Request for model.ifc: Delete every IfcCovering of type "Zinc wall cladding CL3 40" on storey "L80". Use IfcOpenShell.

First a look at what the model holds.

```python
import ifcopenshell
import ifcopenshell.util.element

model = ifcopenshell.open("model.ifc")
print(model.schema)
storey = next(s for s in model.by_type("IfcBuildingStorey") if s.Name == "L80")
coverings = [e for e in ifcopenshell.util.element.get_decomposition(storey) if e.is_a("IfcCovering")]
seen = {}
for e in coverings:
    element_type = ifcopenshell.util.element.get_type(e)
    name = element_type.Name if element_type not in (None, e) else None
    seen[name] = seen.get(name, 0) + 1
for name, count in sorted(seen.items(), key=str):
    print(count, "x", name)
```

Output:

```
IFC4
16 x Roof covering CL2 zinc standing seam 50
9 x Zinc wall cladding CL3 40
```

```python
import ifcopenshell
import ifcopenshell.api.root
import ifcopenshell.util.element

model = ifcopenshell.open("model.ifc")

storey = next(s for s in model.by_type("IfcBuildingStorey") if s.Name == "L80")
coverings = [e for e in ifcopenshell.util.element.get_decomposition(storey) if e.is_a("IfcCovering")]
targets = [e for e in coverings if (t := ifcopenshell.util.element.get_type(e)) not in (None, e) and t.Name == "Zinc wall cladding CL3 40"]

for e in targets:
    ifcopenshell.api.root.remove_product(model, product=e)
print(len(targets), "removed")

model.write("model_updated.ifc")
```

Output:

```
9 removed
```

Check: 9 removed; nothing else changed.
